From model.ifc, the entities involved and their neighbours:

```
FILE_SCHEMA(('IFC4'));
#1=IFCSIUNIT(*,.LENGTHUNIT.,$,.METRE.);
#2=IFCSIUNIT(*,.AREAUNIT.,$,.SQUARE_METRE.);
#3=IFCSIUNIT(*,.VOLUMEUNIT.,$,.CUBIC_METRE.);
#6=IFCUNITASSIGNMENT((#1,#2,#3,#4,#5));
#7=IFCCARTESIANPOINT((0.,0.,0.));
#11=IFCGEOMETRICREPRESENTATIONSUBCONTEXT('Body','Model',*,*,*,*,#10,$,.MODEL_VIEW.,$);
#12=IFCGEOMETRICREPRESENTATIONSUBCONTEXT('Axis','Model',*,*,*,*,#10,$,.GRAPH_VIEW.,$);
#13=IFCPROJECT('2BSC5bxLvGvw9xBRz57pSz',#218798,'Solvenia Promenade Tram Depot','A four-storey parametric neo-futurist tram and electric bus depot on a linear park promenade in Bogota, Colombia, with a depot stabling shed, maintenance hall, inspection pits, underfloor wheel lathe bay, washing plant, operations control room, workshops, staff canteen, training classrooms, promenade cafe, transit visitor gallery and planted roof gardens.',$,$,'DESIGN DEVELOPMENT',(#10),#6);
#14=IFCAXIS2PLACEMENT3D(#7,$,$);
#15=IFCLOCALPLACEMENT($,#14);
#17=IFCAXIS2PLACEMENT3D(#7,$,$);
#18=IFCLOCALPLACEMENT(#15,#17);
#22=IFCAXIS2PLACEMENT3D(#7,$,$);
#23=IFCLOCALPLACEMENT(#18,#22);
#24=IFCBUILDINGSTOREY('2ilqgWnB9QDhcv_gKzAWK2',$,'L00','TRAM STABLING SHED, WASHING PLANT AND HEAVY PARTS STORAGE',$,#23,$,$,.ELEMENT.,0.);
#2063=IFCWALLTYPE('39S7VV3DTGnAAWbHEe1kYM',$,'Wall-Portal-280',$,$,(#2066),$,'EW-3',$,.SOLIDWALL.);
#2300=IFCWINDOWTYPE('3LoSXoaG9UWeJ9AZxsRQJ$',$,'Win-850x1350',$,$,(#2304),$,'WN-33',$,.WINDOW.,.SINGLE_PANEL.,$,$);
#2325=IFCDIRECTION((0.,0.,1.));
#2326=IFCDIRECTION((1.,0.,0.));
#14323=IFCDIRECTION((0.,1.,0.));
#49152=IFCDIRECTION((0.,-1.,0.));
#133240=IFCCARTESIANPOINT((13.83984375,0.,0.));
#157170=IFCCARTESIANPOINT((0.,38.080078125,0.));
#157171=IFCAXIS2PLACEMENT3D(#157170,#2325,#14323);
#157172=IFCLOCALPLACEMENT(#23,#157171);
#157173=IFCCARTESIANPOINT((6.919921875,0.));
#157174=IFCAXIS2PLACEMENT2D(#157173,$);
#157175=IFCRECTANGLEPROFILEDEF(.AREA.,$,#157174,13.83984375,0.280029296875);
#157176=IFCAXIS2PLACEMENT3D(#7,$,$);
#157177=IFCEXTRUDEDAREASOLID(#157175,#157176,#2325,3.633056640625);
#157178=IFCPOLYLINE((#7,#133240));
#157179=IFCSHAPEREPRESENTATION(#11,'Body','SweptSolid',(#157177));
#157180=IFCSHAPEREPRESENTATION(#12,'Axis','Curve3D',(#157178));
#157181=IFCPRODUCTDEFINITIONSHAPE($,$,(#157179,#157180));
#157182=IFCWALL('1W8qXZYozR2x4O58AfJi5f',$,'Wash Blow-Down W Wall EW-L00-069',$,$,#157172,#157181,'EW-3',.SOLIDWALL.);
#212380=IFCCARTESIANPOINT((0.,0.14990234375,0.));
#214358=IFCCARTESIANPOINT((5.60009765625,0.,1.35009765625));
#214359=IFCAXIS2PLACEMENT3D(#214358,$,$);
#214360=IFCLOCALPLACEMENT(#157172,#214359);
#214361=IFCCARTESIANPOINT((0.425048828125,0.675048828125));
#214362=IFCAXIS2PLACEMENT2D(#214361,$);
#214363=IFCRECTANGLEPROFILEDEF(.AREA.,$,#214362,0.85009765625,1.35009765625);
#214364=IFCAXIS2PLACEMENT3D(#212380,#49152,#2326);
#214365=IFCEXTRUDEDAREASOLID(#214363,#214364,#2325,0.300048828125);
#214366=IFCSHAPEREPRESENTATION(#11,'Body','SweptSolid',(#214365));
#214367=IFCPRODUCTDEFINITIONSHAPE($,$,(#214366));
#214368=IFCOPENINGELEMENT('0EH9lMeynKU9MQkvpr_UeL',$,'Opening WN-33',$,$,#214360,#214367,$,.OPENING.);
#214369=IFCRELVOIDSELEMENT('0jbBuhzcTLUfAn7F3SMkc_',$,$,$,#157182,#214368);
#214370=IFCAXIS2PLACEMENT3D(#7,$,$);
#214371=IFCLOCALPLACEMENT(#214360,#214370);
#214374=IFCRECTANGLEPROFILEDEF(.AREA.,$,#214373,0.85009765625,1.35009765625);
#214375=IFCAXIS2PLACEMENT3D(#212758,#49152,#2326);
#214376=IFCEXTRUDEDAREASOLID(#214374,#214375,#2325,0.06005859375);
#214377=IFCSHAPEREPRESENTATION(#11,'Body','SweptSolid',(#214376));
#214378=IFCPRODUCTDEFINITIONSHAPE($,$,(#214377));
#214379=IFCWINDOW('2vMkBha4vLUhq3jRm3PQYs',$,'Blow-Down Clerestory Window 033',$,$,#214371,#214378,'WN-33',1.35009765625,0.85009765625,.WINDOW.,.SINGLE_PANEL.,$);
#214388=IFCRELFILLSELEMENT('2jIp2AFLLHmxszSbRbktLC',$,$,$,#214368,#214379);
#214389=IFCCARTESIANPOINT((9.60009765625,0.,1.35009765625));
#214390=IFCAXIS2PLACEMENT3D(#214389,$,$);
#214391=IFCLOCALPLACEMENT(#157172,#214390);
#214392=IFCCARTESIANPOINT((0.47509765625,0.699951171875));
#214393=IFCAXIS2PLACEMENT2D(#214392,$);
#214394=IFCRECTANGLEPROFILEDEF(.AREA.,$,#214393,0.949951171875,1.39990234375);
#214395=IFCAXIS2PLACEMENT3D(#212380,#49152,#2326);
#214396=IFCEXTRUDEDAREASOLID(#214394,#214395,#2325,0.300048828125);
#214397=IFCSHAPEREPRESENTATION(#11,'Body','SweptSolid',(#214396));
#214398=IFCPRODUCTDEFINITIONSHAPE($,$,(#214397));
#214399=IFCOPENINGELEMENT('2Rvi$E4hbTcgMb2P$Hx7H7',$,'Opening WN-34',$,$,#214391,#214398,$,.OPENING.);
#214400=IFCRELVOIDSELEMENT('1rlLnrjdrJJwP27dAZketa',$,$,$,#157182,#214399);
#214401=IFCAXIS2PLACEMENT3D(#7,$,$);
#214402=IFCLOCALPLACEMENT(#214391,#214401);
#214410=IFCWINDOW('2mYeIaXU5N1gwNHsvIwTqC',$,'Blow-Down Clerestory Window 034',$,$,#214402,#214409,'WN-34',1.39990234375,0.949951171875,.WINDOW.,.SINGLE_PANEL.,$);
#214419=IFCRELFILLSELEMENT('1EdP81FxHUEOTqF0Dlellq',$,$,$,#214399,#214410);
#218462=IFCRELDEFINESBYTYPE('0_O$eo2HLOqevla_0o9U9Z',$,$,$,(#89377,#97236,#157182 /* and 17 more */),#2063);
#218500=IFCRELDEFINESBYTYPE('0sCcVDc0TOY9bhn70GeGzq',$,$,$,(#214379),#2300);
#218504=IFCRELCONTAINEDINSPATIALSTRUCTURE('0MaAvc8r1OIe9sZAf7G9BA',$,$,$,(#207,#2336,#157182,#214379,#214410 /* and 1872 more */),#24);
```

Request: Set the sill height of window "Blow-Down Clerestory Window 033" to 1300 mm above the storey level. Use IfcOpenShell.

```python
import numpy as np
import ifcopenshell
import ifcopenshell.api.geometry
import ifcopenshell.geom
import ifcopenshell.util.element
import ifcopenshell.util.placement
import ifcopenshell.util.shape
import ifcopenshell.util.unit

model = ifcopenshell.open("model.ifc")
unit_scale = ifcopenshell.util.unit.calculate_unit_scale(model)

window = model.by_id(214379)
opening = window.FillsVoids[0].RelatingOpeningElement
storey = ifcopenshell.util.element.get_container(window, ifc_class="IfcBuildingStorey")
level = ifcopenshell.util.placement.get_local_placement(storey.ObjectPlacement)[2, 3]

# The opening's origin need not be at the sill, so measure its lowest point.
shape = ifcopenshell.geom.create_shape(ifcopenshell.geom.settings(), opening)
bottom = ifcopenshell.util.shape.get_shape_bottom_elevation(shape, shape.geometry) / unit_scale
dz = level + 1.3 - bottom

shift = np.array([0.0, 0.0, dz])
# The window is placed relative to its opening, so it follows when the opening moves.
matrix = ifcopenshell.util.placement.get_local_placement(opening.ObjectPlacement)
matrix[:3, 3] += shift
ifcopenshell.api.geometry.edit_object_placement(
    model, product=opening, matrix=matrix, is_si=False, should_transform_children=True
)

print(f"moved by {dz * unit_scale:+.3f} m")

model.write("model_updated.ifc")
```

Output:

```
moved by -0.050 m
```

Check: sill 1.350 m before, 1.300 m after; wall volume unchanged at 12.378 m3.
